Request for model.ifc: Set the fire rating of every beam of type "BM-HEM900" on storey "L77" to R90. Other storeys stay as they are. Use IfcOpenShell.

First a look at what the model holds.

```python
import ifcopenshell
import ifcopenshell.util.element

model = ifcopenshell.open("model.ifc")
print(model.schema)
storey = next(s for s in model.by_type("IfcBuildingStorey") if s.Name == "L77")
beams = [e for e in ifcopenshell.util.element.get_decomposition(storey) if e.is_a("IfcBeam")]
seen = {}
for e in beams:
    element_type = ifcopenshell.util.element.get_type(e)
    key = (element_type.Name if element_type != e and element_type else None, ifcopenshell.util.element.get_pset(e, "Pset_BeamCommon", "FireRating"))
    seen[key] = seen.get(key, 0) + 1
for (name, value), count in sorted(seen.items(), key=str):
    print(count, "x", name, "|", value)
```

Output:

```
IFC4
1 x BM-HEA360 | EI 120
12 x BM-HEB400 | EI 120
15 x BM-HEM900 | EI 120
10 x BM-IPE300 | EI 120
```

```python
import ifcopenshell
import ifcopenshell.api.pset
import ifcopenshell.util.element

model = ifcopenshell.open("model.ifc")

storey = next(s for s in model.by_type("IfcBuildingStorey") if s.Name == "L77")
beams = [e for e in ifcopenshell.util.element.get_decomposition(storey) if e.is_a("IfcBeam")]

count = 0
for e in beams:
    element_type = ifcopenshell.util.element.get_type(e)
    if element_type in (None, e) or element_type.Name != "BM-HEM900":
        continue
    # add_pset returns the element's existing set when there is one.
    pset = ifcopenshell.api.pset.add_pset(model, product=e, name="Pset_BeamCommon")
    ifcopenshell.api.pset.edit_pset(model, pset=pset, properties={"FireRating": "R90"})
    count += 1

print(count, "beams updated")

model.write("model_edited.ifc")
```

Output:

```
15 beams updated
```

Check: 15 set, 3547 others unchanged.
